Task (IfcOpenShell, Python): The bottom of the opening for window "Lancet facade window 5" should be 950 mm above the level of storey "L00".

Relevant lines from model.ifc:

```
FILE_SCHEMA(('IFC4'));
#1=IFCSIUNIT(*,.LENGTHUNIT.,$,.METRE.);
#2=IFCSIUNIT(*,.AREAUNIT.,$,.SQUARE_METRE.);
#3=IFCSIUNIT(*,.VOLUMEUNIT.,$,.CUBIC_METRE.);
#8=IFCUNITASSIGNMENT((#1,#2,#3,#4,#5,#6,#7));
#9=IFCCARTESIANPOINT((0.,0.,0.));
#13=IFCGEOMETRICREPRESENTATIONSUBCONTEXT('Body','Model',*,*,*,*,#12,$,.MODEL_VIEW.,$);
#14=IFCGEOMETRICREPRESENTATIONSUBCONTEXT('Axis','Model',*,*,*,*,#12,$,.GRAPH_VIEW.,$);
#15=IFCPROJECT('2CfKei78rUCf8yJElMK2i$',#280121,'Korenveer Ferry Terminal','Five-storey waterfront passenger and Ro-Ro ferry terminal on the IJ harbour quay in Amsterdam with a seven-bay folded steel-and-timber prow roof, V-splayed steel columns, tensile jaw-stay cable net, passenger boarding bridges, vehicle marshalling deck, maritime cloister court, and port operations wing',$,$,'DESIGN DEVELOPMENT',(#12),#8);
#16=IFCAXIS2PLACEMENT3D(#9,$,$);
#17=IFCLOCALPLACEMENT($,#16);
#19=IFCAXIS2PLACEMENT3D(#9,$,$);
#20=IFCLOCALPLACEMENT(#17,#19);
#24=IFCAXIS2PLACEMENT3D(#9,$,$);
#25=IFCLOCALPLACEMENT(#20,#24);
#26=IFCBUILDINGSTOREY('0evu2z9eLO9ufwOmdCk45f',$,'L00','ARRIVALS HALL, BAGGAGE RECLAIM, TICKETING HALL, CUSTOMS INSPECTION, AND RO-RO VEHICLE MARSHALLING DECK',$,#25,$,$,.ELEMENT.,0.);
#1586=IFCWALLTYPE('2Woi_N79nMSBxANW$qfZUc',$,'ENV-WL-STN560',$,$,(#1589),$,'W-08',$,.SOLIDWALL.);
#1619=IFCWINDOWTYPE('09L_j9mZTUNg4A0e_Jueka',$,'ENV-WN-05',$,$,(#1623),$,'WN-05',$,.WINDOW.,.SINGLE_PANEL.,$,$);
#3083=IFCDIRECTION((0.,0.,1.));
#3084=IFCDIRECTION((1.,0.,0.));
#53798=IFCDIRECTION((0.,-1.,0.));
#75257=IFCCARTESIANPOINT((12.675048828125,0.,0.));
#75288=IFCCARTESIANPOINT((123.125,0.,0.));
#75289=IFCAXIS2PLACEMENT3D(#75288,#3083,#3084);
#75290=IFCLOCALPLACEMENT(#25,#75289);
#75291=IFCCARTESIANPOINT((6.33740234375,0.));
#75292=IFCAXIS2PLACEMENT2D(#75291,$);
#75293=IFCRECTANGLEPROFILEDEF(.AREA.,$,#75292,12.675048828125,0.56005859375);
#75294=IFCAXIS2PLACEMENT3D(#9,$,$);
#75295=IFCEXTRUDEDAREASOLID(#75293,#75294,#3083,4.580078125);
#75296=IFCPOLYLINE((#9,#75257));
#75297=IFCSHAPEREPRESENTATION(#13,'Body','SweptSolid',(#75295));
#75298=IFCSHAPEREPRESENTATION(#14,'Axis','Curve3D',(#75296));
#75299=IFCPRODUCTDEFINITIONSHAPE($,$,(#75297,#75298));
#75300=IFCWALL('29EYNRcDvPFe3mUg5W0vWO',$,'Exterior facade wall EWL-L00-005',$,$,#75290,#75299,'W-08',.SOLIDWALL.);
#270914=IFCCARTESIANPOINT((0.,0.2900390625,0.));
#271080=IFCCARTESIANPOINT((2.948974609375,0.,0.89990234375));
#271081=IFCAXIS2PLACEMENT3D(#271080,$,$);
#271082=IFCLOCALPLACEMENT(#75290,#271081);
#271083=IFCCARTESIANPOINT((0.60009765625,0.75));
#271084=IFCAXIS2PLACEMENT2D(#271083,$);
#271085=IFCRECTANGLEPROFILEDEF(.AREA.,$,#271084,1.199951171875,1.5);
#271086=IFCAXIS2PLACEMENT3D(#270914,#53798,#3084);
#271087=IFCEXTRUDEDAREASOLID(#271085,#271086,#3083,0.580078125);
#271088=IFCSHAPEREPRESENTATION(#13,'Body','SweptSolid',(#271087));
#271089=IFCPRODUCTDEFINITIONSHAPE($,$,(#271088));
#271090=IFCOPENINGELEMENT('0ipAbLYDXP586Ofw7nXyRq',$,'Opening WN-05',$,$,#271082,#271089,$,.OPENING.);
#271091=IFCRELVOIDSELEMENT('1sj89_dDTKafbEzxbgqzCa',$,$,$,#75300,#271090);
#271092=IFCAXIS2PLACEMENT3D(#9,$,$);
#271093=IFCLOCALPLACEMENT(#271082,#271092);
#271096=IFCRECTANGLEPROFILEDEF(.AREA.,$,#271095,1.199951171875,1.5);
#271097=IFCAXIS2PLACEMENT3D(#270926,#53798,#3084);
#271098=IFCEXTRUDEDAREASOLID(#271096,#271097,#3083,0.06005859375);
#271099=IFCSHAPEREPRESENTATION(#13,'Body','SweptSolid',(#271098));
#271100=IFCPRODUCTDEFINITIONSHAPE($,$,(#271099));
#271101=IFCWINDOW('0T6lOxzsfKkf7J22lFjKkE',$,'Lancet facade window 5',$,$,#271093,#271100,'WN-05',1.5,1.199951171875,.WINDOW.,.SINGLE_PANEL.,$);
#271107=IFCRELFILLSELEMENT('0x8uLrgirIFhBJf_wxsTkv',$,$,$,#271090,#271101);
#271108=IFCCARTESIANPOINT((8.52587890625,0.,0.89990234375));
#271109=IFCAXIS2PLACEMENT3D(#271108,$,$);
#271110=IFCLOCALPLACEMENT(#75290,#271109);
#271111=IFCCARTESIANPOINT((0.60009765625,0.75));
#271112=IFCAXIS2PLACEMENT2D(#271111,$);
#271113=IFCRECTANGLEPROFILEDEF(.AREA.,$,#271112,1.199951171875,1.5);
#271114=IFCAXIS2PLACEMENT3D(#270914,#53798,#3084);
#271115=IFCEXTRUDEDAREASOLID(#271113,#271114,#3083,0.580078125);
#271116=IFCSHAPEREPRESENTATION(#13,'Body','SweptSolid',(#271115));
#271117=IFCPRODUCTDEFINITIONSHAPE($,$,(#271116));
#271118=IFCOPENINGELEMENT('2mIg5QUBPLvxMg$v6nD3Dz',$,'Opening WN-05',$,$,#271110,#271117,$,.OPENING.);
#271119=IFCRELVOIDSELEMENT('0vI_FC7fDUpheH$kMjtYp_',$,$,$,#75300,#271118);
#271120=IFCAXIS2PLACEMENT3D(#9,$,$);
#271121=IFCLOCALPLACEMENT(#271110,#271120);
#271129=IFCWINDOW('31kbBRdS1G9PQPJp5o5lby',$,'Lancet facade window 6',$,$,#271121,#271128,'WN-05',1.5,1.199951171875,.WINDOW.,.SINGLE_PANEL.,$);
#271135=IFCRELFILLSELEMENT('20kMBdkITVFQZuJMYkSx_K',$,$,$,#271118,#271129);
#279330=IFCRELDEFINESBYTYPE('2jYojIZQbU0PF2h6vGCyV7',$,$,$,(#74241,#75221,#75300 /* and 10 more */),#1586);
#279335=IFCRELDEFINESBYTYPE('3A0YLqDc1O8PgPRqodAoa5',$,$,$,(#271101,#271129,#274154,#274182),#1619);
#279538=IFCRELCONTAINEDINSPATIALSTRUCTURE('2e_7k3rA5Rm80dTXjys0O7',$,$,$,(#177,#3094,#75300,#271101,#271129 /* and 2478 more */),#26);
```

```python
import numpy as np
import ifcopenshell
import ifcopenshell.api.geometry
import ifcopenshell.geom
import ifcopenshell.util.element
import ifcopenshell.util.placement
import ifcopenshell.util.shape
import ifcopenshell.util.unit

model = ifcopenshell.open("model.ifc")
unit_scale = ifcopenshell.util.unit.calculate_unit_scale(model)

window = model.by_guid("0T6lOxzsfKkf7J22lFjKkE")
opening = window.FillsVoids[0].RelatingOpeningElement
storey = ifcopenshell.util.element.get_container(window, ifc_class="IfcBuildingStorey")
level = ifcopenshell.util.placement.get_local_placement(storey.ObjectPlacement)[2, 3]

# The opening's origin need not be at the sill, so measure its lowest point.
shape = ifcopenshell.geom.create_shape(ifcopenshell.geom.settings(), opening)
bottom = ifcopenshell.util.shape.get_shape_bottom_elevation(shape, shape.geometry) / unit_scale
dz = level + 0.95 - bottom

shift = np.array([0.0, 0.0, dz])
# The window is placed relative to its opening, so it follows when the opening moves.
matrix = ifcopenshell.util.placement.get_local_placement(opening.ObjectPlacement)
matrix[:3, 3] += shift
ifcopenshell.api.geometry.edit_object_placement(
    model, product=opening, matrix=matrix, is_si=False, should_transform_children=True
)

print(f"moved by {dz * unit_scale:+.3f} m")

model.write("model_edited.ifc")
```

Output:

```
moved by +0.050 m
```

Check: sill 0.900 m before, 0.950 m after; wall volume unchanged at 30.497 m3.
